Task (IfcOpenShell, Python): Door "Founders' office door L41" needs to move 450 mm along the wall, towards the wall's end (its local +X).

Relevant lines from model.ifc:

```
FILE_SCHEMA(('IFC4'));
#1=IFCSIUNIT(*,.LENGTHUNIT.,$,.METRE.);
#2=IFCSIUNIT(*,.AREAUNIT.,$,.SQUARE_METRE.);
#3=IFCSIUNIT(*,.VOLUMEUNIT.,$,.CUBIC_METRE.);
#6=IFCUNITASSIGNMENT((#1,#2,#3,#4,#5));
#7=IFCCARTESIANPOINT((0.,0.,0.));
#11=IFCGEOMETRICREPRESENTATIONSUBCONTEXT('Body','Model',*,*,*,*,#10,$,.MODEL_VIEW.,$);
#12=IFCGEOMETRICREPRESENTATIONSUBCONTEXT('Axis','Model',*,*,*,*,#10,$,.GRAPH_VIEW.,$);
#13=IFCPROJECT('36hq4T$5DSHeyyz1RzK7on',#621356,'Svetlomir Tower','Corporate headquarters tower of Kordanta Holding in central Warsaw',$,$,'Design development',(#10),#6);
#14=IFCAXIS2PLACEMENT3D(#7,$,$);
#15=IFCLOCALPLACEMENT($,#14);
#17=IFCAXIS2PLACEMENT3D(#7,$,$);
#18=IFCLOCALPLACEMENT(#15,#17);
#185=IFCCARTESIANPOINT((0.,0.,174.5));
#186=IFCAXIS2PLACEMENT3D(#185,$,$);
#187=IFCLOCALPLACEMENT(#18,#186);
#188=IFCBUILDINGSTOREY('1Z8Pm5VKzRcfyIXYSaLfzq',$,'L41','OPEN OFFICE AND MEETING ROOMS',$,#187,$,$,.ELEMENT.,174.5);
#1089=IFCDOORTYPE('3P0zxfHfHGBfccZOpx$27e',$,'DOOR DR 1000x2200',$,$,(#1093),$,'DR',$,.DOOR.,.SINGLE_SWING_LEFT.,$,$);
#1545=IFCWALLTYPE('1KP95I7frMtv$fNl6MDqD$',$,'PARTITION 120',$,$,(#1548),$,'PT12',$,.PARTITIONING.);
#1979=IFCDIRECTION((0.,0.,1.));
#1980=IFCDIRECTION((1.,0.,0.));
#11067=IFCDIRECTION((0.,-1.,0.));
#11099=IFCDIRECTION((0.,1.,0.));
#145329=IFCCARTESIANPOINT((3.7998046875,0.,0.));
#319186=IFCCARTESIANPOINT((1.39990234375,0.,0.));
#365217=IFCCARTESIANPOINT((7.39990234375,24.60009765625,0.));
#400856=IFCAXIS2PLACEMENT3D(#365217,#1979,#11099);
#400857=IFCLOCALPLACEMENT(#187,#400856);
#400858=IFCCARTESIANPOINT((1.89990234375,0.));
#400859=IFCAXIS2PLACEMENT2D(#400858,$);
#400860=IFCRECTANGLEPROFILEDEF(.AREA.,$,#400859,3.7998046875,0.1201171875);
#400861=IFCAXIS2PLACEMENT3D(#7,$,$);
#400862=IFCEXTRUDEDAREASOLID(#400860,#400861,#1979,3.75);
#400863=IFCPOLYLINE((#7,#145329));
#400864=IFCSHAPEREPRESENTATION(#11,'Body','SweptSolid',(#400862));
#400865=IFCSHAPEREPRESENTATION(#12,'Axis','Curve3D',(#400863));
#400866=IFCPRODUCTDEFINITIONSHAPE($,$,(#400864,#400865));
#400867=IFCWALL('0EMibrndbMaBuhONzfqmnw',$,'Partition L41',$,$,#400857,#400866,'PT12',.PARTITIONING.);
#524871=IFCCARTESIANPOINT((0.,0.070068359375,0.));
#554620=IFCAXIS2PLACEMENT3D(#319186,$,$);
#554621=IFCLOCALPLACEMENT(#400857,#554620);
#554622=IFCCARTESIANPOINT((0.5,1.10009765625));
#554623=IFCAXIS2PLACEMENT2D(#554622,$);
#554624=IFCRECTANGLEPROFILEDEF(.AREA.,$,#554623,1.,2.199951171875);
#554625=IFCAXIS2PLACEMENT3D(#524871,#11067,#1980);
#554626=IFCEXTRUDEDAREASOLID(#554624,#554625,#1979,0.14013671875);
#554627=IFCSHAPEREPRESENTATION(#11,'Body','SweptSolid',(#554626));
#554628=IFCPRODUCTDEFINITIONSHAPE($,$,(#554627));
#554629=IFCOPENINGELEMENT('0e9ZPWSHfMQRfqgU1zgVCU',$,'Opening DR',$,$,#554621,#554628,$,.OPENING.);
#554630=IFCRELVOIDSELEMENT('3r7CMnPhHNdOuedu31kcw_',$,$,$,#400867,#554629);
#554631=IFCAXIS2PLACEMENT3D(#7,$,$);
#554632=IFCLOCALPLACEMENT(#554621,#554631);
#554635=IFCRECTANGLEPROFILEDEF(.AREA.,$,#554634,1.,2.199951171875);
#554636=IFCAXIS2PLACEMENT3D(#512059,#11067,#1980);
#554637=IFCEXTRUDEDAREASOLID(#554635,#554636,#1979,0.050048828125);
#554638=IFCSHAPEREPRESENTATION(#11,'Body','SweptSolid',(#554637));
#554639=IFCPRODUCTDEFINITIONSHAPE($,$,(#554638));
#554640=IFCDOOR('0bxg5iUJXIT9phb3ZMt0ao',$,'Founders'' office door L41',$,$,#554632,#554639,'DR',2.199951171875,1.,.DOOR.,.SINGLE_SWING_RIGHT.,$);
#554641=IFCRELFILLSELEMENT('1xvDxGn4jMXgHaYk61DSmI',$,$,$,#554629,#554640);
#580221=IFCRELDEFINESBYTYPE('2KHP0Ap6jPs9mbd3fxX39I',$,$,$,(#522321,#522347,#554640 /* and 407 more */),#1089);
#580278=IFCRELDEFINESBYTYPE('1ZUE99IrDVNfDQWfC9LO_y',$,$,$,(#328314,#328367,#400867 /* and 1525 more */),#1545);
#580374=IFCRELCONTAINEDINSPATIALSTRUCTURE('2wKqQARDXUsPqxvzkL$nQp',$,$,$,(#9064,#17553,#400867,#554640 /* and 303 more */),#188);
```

```python
import ifcopenshell
import ifcopenshell.api.geometry
import ifcopenshell.util.placement
import ifcopenshell.util.unit

model = ifcopenshell.open("model.ifc")
unit_scale = ifcopenshell.util.unit.calculate_unit_scale(model)

door = model.by_guid("0bxg5iUJXIT9phb3ZMt0ao")
opening = door.FillsVoids[0].RelatingOpeningElement
wall = opening.VoidsElements[0].RelatingBuildingElement

wall_matrix = ifcopenshell.util.placement.get_local_placement(wall.ObjectPlacement)
shift = wall_matrix[:3, 0] * 0.45 / unit_scale
before = ifcopenshell.util.placement.get_local_placement(door.ObjectPlacement)[:3, 3].copy()

# The door is placed relative to its opening, so it follows when the opening moves.
matrix = ifcopenshell.util.placement.get_local_placement(opening.ObjectPlacement)
matrix[:3, 3] += shift
ifcopenshell.api.geometry.edit_object_placement(
    model, product=opening, matrix=matrix, is_si=False, should_transform_children=True
)

after = ifcopenshell.util.placement.get_local_placement(door.ObjectPlacement)[:3, 3]
print("door moved by", (after - before).round(3) + 0.0)

model.write("model_updated.ifc")
```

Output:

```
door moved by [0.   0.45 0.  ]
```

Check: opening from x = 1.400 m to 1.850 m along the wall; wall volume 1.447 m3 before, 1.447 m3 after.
